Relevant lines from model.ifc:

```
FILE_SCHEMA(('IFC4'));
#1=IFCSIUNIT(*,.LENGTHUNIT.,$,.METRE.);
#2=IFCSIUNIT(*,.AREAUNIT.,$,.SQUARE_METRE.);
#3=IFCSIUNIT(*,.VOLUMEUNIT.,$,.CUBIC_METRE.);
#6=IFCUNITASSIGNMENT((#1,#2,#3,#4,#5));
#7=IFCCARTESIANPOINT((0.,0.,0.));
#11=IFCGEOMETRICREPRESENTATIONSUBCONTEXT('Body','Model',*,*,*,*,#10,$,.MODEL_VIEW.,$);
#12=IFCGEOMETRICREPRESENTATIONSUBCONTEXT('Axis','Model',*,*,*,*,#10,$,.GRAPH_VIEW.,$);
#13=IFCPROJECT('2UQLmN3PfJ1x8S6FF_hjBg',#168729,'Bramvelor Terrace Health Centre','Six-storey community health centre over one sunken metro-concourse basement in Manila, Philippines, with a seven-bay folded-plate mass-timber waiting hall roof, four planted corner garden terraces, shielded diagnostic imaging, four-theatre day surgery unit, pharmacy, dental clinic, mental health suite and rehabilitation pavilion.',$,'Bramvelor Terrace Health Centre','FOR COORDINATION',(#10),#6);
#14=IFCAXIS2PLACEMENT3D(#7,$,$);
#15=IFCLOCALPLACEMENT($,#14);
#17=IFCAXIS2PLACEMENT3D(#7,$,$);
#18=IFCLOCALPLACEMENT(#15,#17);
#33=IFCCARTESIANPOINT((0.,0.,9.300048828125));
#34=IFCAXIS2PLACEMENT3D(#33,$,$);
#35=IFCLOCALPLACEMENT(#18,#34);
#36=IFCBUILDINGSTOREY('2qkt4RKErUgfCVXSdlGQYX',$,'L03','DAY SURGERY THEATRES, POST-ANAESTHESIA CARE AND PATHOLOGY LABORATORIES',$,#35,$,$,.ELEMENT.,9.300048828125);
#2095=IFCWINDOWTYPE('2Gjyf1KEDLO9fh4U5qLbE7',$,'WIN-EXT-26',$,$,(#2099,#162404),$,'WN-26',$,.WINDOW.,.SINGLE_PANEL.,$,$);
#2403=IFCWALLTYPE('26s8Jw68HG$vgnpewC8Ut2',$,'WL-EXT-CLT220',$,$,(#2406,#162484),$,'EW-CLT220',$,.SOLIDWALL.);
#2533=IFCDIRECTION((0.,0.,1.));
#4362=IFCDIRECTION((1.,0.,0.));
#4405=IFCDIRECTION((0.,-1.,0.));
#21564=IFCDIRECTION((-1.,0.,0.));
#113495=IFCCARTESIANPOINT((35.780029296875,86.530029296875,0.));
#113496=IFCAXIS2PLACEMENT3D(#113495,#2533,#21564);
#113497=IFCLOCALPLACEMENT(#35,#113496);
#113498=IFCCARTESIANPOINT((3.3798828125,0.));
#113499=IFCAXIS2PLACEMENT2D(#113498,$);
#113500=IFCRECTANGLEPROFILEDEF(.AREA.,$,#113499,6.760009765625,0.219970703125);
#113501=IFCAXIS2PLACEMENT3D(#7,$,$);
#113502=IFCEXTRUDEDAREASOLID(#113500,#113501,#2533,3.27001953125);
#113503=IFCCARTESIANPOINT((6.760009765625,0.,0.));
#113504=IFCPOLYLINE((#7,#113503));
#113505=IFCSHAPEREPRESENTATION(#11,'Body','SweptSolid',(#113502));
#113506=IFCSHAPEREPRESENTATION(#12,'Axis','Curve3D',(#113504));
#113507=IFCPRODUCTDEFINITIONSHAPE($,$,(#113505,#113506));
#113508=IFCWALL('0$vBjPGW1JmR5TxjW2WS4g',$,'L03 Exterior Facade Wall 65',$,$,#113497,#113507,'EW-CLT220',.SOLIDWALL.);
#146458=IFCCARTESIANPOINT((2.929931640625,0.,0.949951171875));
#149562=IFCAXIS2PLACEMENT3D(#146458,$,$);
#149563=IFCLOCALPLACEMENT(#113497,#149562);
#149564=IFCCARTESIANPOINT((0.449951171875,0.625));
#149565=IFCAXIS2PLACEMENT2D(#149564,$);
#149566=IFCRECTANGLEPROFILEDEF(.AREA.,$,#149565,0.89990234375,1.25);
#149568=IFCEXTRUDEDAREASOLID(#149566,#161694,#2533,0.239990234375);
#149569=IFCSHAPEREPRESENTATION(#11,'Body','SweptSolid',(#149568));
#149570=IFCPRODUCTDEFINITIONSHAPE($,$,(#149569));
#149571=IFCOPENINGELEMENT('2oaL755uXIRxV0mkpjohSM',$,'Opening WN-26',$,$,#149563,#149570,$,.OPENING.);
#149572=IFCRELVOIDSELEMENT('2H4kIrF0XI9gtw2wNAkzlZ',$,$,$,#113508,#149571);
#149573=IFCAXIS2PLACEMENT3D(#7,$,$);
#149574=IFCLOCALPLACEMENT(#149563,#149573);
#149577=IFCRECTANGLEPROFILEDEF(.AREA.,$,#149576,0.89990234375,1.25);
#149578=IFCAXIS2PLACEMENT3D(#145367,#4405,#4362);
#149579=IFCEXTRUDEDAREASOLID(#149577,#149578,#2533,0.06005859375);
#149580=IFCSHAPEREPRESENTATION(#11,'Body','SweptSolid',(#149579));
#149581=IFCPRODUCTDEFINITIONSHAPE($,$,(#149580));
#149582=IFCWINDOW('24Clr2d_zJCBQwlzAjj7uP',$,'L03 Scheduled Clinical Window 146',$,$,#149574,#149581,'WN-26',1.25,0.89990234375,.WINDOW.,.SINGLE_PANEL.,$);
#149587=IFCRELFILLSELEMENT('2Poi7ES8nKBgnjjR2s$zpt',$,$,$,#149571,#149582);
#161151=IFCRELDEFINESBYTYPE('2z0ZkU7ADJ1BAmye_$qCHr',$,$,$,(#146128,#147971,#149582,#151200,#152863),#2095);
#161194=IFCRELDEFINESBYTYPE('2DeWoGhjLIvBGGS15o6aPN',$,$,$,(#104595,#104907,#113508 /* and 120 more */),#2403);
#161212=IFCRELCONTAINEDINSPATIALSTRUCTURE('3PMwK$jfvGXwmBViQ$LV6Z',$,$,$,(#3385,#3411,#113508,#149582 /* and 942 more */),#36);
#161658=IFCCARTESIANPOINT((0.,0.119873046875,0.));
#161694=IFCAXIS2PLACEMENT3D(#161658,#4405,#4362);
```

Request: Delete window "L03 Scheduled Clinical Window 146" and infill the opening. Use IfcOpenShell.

```python
import ifcopenshell
import ifcopenshell.api.feature
import ifcopenshell.api.root
import ifcopenshell.geom
import ifcopenshell.util.shape

model = ifcopenshell.open("model.ifc")
settings = ifcopenshell.geom.settings()


def volume(element):
    """Net volume in cubic metres, openings subtracted."""
    shape = ifcopenshell.geom.create_shape(settings, element)
    return ifcopenshell.util.shape.get_volume(shape.geometry)


window = model.by_guid("24Clr2d_zJCBQwlzAjj7uP")
opening = window.FillsVoids[0].RelatingOpeningElement
wall = opening.VoidsElements[0].RelatingBuildingElement
before = volume(wall)

ifcopenshell.api.root.remove_product(model, product=window)
ifcopenshell.api.feature.remove_feature(model, feature=opening)

after = volume(wall)

print(f"wall volume {before:.3f} -> {after:.3f} m3")

model.write("model_updated.ifc")
```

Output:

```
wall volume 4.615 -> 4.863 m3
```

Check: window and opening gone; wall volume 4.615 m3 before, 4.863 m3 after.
